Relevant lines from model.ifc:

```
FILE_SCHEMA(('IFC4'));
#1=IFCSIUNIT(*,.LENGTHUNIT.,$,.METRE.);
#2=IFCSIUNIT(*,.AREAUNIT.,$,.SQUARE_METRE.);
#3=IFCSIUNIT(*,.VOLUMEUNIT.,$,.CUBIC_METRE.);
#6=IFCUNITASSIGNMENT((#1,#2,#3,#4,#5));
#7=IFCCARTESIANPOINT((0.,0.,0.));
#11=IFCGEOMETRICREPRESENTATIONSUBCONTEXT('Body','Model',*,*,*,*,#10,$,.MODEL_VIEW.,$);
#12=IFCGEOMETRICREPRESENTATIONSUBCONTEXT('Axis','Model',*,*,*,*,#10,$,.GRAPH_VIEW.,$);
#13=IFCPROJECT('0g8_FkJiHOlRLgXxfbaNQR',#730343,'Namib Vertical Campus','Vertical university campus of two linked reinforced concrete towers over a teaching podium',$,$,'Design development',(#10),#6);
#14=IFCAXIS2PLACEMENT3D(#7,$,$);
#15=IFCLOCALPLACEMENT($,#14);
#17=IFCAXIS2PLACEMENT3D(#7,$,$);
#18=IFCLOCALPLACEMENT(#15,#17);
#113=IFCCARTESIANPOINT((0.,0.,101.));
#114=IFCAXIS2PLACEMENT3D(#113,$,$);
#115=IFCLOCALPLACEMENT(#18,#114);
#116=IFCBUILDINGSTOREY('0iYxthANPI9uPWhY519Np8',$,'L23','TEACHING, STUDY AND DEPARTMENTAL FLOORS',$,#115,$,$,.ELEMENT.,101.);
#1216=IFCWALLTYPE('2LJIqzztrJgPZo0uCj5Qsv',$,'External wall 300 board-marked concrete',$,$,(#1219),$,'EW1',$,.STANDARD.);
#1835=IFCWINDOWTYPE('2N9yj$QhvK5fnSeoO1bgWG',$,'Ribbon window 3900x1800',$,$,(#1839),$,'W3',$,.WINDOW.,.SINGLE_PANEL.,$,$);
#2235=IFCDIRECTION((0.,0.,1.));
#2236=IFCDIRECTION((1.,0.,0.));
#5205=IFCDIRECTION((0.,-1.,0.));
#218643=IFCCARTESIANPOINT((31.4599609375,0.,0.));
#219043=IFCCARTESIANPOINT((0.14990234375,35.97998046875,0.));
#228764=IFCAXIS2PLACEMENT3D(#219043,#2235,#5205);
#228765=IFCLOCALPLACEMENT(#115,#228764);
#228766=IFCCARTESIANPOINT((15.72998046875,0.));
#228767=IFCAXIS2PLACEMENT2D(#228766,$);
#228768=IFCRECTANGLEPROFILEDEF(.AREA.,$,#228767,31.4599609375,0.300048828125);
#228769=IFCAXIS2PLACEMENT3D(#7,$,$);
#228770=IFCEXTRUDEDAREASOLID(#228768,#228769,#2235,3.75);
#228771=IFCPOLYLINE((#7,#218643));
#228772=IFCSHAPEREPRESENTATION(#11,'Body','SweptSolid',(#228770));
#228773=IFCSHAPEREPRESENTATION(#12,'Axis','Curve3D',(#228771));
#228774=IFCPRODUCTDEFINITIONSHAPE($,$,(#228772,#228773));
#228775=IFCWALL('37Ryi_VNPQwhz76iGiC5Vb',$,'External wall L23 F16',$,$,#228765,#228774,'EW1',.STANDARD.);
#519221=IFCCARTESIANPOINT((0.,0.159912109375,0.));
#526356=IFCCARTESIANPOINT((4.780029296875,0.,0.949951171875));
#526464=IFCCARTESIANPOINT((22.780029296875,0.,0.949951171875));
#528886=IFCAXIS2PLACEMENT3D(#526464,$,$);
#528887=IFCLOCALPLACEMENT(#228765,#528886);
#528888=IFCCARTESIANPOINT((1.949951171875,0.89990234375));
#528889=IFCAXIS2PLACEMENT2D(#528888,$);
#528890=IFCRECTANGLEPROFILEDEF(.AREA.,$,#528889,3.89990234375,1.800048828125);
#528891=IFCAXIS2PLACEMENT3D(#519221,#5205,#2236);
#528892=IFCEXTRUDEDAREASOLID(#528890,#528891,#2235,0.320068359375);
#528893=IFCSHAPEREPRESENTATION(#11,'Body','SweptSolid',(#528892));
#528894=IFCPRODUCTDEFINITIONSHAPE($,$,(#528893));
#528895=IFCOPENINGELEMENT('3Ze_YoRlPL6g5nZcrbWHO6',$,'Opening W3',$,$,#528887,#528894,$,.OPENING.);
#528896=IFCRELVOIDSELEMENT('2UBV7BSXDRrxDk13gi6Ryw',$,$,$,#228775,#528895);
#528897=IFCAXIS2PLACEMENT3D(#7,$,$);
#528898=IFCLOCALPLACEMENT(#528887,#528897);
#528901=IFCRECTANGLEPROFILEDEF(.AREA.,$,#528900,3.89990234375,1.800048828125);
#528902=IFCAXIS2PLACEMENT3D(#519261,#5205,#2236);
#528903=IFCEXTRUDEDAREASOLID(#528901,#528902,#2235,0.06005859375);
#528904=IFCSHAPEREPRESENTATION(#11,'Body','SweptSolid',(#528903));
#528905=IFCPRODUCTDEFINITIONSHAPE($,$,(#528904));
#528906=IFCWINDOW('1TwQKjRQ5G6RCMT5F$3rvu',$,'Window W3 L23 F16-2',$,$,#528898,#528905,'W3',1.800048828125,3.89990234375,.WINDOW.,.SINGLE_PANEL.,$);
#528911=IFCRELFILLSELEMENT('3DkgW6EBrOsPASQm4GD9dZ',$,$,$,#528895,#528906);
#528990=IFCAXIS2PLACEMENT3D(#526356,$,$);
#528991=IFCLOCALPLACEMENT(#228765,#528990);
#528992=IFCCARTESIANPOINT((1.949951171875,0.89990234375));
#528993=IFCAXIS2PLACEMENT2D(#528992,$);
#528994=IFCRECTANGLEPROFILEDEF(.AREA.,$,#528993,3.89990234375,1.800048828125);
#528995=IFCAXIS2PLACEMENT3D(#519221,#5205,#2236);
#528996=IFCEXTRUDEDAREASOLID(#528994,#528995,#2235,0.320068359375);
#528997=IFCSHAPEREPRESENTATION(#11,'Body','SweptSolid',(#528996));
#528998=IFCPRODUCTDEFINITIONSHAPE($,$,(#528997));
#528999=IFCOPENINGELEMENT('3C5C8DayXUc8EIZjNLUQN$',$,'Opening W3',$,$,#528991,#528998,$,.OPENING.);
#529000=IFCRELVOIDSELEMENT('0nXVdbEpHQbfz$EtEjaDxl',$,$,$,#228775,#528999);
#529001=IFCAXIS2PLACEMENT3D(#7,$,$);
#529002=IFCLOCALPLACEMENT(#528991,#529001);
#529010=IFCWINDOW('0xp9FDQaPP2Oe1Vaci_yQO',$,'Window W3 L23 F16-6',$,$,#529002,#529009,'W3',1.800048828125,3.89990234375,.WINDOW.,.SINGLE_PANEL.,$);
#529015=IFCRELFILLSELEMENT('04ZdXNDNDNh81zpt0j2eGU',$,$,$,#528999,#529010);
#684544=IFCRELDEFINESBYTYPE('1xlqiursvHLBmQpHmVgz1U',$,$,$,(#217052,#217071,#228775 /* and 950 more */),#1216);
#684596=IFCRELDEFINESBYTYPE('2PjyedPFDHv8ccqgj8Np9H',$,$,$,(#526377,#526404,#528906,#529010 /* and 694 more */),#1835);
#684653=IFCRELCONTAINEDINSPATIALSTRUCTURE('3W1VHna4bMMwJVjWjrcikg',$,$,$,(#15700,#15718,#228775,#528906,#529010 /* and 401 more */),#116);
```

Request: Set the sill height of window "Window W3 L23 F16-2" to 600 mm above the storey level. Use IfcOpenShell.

```python
import numpy as np
import ifcopenshell
import ifcopenshell.api.geometry
import ifcopenshell.geom
import ifcopenshell.util.element
import ifcopenshell.util.placement
import ifcopenshell.util.shape
import ifcopenshell.util.unit

model = ifcopenshell.open("model.ifc")
unit_scale = ifcopenshell.util.unit.calculate_unit_scale(model)

window = model.by_id(528906)
opening = window.FillsVoids[0].RelatingOpeningElement
storey = ifcopenshell.util.element.get_container(window, ifc_class="IfcBuildingStorey")
level = ifcopenshell.util.placement.get_local_placement(storey.ObjectPlacement)[2, 3]

# The opening's origin need not be at the sill, so measure its lowest point.
shape = ifcopenshell.geom.create_shape(ifcopenshell.geom.settings(), opening)
bottom = ifcopenshell.util.shape.get_shape_bottom_elevation(shape, shape.geometry) / unit_scale
dz = level + 0.6 / unit_scale - bottom

shift = np.array([0.0, 0.0, dz])
# The window is placed relative to its opening, so it follows when the opening moves.
matrix = ifcopenshell.util.placement.get_local_placement(opening.ObjectPlacement)
matrix[:3, 3] += shift
ifcopenshell.api.geometry.edit_object_placement(
    model, product=opening, matrix=matrix, is_si=False, should_transform_children=True
)

print(f"moved by {dz * unit_scale:+.3f} m")

model.write("model-out.ifc")
```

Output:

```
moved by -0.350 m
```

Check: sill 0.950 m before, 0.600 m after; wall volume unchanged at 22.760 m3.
